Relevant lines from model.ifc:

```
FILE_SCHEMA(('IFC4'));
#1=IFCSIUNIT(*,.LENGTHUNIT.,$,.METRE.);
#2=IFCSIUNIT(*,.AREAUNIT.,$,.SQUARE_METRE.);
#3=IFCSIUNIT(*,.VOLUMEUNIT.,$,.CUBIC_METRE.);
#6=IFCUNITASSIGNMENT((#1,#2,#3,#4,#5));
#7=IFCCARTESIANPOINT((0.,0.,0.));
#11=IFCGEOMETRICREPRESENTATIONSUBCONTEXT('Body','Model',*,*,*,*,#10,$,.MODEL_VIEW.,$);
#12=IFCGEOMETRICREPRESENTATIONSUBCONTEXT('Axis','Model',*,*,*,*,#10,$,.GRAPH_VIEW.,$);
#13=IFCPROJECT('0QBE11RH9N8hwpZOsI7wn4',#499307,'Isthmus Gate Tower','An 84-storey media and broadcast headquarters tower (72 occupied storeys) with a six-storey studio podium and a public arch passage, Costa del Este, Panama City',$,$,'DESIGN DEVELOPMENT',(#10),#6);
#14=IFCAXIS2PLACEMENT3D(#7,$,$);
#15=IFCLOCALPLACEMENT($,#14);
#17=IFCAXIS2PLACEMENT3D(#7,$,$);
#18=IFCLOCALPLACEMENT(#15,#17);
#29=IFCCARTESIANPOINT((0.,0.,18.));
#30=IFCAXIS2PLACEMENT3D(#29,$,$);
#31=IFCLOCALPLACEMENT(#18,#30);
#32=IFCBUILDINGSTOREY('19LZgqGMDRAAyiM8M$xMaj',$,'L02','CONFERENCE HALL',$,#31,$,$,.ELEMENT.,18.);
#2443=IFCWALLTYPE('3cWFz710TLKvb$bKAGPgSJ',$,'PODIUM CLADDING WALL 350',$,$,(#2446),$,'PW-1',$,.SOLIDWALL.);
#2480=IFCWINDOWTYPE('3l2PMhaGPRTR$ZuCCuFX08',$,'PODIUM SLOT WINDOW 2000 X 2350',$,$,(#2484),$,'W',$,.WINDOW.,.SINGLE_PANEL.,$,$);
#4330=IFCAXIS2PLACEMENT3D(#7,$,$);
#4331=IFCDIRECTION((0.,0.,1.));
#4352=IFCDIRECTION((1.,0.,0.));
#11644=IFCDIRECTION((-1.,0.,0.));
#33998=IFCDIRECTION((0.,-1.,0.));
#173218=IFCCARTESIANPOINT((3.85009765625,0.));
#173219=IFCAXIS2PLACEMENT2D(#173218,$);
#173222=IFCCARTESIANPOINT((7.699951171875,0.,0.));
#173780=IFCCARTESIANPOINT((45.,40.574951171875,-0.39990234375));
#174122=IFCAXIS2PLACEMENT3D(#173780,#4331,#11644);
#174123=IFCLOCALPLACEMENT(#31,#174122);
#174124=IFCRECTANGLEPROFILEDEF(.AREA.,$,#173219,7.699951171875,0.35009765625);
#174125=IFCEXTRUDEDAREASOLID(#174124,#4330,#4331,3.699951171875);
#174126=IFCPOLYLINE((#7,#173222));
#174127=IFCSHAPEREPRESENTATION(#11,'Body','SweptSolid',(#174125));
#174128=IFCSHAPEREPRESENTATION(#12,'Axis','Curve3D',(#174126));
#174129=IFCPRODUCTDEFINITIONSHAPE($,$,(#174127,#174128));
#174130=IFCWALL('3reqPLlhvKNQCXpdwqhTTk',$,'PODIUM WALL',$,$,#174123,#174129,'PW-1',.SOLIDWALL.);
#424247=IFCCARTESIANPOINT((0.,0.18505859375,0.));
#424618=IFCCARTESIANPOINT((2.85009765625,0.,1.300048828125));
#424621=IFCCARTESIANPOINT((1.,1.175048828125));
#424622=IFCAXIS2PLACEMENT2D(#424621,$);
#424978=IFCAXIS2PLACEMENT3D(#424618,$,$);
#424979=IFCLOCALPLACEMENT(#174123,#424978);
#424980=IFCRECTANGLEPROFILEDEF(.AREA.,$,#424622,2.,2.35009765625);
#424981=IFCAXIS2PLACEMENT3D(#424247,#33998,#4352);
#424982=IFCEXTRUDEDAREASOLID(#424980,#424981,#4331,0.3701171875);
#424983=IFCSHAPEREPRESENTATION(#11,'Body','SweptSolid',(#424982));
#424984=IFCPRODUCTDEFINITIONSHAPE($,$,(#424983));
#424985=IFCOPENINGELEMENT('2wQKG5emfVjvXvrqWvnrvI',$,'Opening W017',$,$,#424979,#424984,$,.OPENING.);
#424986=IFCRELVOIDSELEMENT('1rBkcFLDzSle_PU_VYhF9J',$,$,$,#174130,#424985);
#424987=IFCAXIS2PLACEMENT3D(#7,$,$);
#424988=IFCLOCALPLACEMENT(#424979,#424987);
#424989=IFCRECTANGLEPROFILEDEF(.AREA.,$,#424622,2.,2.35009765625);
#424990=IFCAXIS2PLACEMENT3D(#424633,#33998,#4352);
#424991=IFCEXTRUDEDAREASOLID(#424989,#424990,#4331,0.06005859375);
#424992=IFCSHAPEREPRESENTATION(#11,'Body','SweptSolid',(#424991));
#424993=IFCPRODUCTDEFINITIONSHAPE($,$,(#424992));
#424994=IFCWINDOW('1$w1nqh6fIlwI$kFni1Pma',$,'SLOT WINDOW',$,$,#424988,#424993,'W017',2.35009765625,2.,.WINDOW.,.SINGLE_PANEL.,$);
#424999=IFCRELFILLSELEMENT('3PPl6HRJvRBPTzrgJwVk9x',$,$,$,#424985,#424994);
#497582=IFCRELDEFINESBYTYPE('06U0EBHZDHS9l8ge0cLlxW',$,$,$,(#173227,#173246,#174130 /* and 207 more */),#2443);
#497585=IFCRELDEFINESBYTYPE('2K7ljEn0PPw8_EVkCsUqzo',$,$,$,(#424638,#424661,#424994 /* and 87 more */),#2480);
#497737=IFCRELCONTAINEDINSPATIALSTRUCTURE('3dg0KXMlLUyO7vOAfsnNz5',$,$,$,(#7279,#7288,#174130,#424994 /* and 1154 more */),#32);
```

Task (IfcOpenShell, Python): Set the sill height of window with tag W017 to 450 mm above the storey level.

```python
import numpy as np
import ifcopenshell
import ifcopenshell.api.geometry
import ifcopenshell.geom
import ifcopenshell.util.element
import ifcopenshell.util.placement
import ifcopenshell.util.shape
import ifcopenshell.util.unit

model = ifcopenshell.open("model.ifc")
unit_scale = ifcopenshell.util.unit.calculate_unit_scale(model)

window = model.by_guid("1$w1nqh6fIlwI$kFni1Pma")
opening = window.FillsVoids[0].RelatingOpeningElement
storey = ifcopenshell.util.element.get_container(window, ifc_class="IfcBuildingStorey")
level = ifcopenshell.util.placement.get_local_placement(storey.ObjectPlacement)[2, 3]

# The opening's origin need not be at the sill, so measure its lowest point.
shape = ifcopenshell.geom.create_shape(ifcopenshell.geom.settings(), opening)
bottom = ifcopenshell.util.shape.get_shape_bottom_elevation(shape, shape.geometry) / unit_scale
dz = level + 0.45 / unit_scale - bottom

shift = np.array([0.0, 0.0, dz])
# The window is placed relative to its opening, so it follows when the opening moves.
matrix = ifcopenshell.util.placement.get_local_placement(opening.ObjectPlacement)
matrix[:3, 3] += shift
ifcopenshell.api.geometry.edit_object_placement(
    model, product=opening, matrix=matrix, is_si=False, should_transform_children=True
)

print(f"moved by {dz * unit_scale:+.3f} m")

model.write("model_rev.ifc")
```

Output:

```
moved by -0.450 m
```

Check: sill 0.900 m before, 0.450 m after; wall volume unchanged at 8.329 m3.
